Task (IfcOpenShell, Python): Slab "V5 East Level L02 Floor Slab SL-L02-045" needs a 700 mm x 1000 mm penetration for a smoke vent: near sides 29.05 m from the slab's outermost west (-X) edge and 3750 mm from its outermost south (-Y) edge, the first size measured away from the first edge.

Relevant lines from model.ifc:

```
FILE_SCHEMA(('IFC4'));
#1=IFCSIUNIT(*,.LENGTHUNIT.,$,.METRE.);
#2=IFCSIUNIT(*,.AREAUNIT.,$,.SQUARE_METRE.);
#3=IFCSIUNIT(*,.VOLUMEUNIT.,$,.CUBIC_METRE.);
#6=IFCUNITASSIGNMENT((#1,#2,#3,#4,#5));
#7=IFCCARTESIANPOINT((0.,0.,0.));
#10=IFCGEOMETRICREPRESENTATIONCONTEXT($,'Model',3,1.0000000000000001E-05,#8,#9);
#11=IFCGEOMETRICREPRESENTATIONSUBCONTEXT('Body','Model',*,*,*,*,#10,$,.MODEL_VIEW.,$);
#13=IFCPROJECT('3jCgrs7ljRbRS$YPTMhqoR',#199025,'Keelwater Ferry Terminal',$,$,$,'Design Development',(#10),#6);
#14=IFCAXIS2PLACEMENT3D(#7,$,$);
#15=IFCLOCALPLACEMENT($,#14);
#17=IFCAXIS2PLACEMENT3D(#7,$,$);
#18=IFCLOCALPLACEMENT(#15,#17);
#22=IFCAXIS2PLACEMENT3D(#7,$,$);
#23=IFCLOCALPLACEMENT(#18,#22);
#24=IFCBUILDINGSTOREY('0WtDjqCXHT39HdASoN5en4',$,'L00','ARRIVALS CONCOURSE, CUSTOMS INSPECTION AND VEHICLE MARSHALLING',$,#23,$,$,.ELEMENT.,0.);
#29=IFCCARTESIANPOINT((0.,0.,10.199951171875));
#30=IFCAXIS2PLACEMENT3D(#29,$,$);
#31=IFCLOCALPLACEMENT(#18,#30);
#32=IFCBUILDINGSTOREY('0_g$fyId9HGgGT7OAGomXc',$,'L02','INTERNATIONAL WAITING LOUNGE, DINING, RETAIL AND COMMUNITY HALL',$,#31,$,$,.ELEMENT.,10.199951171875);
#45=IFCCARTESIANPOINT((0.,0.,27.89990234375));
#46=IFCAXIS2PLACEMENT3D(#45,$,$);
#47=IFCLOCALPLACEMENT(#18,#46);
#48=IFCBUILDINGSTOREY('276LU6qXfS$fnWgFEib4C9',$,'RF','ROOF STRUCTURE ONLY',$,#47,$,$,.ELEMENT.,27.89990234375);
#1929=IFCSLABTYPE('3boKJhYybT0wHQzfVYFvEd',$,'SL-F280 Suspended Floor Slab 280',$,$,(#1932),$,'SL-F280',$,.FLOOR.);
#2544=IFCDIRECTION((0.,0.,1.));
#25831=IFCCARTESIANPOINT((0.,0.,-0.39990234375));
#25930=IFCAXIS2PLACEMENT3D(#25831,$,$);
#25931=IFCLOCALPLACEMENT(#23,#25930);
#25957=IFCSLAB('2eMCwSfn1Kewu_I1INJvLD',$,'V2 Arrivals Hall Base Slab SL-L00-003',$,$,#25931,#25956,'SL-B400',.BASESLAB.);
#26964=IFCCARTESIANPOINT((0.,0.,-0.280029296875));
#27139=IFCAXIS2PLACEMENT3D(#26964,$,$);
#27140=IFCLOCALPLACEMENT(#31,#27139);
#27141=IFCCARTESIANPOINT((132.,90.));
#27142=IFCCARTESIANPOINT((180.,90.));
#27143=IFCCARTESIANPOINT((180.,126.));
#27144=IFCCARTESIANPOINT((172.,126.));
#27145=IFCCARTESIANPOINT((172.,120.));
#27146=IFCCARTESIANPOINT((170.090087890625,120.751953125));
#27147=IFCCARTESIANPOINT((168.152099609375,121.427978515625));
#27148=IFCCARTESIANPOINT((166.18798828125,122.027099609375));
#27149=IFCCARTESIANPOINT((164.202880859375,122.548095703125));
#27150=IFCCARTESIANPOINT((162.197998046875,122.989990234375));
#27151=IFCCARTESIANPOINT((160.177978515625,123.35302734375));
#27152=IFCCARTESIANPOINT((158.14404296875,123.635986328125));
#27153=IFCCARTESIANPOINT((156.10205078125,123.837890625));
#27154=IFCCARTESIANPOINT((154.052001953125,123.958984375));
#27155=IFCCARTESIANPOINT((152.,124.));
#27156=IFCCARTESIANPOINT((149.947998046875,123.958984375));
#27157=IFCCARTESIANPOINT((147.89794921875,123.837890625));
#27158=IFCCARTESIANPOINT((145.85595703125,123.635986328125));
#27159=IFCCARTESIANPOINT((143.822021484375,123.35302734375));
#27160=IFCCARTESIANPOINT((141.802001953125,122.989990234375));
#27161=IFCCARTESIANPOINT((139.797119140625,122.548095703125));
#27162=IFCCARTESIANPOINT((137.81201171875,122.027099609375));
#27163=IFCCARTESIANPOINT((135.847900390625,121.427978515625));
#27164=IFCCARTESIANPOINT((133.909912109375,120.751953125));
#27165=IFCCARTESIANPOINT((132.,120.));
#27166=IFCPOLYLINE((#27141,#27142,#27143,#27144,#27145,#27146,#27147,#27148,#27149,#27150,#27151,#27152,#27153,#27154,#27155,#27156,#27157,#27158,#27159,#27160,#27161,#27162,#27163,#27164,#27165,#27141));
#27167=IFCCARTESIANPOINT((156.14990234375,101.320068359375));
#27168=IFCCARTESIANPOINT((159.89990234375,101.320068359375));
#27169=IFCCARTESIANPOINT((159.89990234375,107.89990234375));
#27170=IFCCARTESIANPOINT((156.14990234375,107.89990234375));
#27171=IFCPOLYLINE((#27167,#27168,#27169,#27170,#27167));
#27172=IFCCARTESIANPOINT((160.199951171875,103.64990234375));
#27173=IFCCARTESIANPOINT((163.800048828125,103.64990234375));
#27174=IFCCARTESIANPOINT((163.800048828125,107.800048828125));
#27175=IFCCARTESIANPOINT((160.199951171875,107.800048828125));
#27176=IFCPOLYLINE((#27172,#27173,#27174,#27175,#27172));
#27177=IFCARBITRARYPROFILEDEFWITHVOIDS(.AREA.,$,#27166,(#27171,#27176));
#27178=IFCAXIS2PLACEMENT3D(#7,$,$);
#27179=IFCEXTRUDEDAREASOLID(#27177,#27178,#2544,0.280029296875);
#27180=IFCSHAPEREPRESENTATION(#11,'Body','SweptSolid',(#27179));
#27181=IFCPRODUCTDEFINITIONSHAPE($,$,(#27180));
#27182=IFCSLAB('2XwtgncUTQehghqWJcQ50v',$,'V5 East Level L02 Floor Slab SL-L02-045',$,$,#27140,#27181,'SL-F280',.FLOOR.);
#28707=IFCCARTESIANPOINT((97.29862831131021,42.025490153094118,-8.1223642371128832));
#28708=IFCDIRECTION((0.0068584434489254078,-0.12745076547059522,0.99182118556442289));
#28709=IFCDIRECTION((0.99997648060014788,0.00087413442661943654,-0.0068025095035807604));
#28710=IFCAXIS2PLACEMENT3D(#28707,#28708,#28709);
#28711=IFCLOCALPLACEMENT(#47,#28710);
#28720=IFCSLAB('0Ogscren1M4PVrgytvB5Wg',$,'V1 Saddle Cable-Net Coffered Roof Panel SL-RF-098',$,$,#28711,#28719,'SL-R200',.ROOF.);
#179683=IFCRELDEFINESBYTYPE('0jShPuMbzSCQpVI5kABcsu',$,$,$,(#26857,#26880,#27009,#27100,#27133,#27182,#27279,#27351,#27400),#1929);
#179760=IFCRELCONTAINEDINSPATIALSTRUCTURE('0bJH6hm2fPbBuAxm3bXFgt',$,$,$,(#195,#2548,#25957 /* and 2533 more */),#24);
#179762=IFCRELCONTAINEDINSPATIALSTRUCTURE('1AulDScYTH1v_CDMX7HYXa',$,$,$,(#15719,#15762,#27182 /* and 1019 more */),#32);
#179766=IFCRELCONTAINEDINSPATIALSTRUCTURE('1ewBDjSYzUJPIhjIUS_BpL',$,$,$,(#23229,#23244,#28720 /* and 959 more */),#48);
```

```python
import numpy as np
import ifcopenshell
import ifcopenshell.api.feature
import ifcopenshell.api.geometry
import ifcopenshell.api.root
import ifcopenshell.geom
import ifcopenshell.util.placement
import ifcopenshell.util.representation
import ifcopenshell.util.shape
import ifcopenshell.util.unit

model = ifcopenshell.open("model.ifc")
unit_scale = ifcopenshell.util.unit.calculate_unit_scale(model)
settings = ifcopenshell.geom.settings()


def volume(element):
    """Net volume in cubic metres, openings subtracted."""
    shape = ifcopenshell.geom.create_shape(settings, element)
    return ifcopenshell.util.shape.get_volume(shape.geometry)


slab = model.by_id(27182)
before = volume(slab)

# Extent in the slab's own axes, in metres. The edges named are its -X and -Y sides.
slab_shape = ifcopenshell.geom.create_shape(settings, slab)
vertices = ifcopenshell.util.shape.get_vertices(slab_shape.geometry)
x_min, y_min, bottom = vertices.min(axis=0)
top = vertices[:, 2].max()

opening = ifcopenshell.api.root.create_entity(model, ifc_class="IfcOpeningElement", name="Smoke vent opening", predefined_type="OPENING")
context = ifcopenshell.util.representation.get_context(model, "Model", "Body", "MODEL_VIEW")
width, depth = 0.7, 1
outline = [(0.0, 0.0), (width, 0.0), (width, depth), (0.0, depth), (0.0, 0.0)]
# Overshoot both faces by 50 mm so the cut is clean.
shape = ifcopenshell.api.geometry.add_slab_representation(
    model, context=context, depth=top - bottom + 0.1, polyline=outline
)
ifcopenshell.api.geometry.assign_representation(model, product=opening, representation=shape)

matrix = ifcopenshell.util.placement.get_local_placement(slab.ObjectPlacement)
matrix[:, 3] = matrix @ np.append(np.array([x_min + 29.05, y_min + 3.75, bottom - 0.05]) / unit_scale, 1.0)
ifcopenshell.api.geometry.edit_object_placement(model, product=opening, matrix=matrix, is_si=False)
ifcopenshell.api.feature.add_feature(model, feature=opening, element=slab)

after = volume(slab)

print(f"slab volume {before:.3f} -> {after:.3f} m3")

model.write("model_updated.ifc")
```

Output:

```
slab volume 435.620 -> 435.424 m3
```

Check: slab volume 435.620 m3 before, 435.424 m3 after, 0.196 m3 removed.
